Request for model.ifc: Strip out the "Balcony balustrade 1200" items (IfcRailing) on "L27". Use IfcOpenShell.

First a look at what the model holds.

```python
import ifcopenshell
import ifcopenshell.util.element

model = ifcopenshell.open("model.ifc")
print(model.schema)
storey = next(s for s in model.by_type("IfcBuildingStorey") if s.Name == "L27")
railings = [e for e in ifcopenshell.util.element.get_decomposition(storey) if e.is_a("IfcRailing")]
seen = {}
for e in railings:
    element_type = ifcopenshell.util.element.get_type(e)
    name = element_type.Name if element_type not in (None, e) else None
    seen[name] = seen.get(name, 0) + 1
for name, count in sorted(seen.items(), key=str):
    print(count, "x", name)
```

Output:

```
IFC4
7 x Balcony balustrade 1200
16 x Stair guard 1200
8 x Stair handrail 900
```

```python
import ifcopenshell
import ifcopenshell.api.root
import ifcopenshell.util.element

model = ifcopenshell.open("model.ifc")

storey = next(s for s in model.by_type("IfcBuildingStorey") if s.Name == "L27")
railings = [e for e in ifcopenshell.util.element.get_decomposition(storey) if e.is_a("IfcRailing")]
targets = [e for e in railings if (t := ifcopenshell.util.element.get_type(e)) not in (None, e) and t.Name == "Balcony balustrade 1200"]

for e in targets:
    ifcopenshell.api.root.remove_product(model, product=e)
print(len(targets), "removed")

model.write("model_edited.ifc")
```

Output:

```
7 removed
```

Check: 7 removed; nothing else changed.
